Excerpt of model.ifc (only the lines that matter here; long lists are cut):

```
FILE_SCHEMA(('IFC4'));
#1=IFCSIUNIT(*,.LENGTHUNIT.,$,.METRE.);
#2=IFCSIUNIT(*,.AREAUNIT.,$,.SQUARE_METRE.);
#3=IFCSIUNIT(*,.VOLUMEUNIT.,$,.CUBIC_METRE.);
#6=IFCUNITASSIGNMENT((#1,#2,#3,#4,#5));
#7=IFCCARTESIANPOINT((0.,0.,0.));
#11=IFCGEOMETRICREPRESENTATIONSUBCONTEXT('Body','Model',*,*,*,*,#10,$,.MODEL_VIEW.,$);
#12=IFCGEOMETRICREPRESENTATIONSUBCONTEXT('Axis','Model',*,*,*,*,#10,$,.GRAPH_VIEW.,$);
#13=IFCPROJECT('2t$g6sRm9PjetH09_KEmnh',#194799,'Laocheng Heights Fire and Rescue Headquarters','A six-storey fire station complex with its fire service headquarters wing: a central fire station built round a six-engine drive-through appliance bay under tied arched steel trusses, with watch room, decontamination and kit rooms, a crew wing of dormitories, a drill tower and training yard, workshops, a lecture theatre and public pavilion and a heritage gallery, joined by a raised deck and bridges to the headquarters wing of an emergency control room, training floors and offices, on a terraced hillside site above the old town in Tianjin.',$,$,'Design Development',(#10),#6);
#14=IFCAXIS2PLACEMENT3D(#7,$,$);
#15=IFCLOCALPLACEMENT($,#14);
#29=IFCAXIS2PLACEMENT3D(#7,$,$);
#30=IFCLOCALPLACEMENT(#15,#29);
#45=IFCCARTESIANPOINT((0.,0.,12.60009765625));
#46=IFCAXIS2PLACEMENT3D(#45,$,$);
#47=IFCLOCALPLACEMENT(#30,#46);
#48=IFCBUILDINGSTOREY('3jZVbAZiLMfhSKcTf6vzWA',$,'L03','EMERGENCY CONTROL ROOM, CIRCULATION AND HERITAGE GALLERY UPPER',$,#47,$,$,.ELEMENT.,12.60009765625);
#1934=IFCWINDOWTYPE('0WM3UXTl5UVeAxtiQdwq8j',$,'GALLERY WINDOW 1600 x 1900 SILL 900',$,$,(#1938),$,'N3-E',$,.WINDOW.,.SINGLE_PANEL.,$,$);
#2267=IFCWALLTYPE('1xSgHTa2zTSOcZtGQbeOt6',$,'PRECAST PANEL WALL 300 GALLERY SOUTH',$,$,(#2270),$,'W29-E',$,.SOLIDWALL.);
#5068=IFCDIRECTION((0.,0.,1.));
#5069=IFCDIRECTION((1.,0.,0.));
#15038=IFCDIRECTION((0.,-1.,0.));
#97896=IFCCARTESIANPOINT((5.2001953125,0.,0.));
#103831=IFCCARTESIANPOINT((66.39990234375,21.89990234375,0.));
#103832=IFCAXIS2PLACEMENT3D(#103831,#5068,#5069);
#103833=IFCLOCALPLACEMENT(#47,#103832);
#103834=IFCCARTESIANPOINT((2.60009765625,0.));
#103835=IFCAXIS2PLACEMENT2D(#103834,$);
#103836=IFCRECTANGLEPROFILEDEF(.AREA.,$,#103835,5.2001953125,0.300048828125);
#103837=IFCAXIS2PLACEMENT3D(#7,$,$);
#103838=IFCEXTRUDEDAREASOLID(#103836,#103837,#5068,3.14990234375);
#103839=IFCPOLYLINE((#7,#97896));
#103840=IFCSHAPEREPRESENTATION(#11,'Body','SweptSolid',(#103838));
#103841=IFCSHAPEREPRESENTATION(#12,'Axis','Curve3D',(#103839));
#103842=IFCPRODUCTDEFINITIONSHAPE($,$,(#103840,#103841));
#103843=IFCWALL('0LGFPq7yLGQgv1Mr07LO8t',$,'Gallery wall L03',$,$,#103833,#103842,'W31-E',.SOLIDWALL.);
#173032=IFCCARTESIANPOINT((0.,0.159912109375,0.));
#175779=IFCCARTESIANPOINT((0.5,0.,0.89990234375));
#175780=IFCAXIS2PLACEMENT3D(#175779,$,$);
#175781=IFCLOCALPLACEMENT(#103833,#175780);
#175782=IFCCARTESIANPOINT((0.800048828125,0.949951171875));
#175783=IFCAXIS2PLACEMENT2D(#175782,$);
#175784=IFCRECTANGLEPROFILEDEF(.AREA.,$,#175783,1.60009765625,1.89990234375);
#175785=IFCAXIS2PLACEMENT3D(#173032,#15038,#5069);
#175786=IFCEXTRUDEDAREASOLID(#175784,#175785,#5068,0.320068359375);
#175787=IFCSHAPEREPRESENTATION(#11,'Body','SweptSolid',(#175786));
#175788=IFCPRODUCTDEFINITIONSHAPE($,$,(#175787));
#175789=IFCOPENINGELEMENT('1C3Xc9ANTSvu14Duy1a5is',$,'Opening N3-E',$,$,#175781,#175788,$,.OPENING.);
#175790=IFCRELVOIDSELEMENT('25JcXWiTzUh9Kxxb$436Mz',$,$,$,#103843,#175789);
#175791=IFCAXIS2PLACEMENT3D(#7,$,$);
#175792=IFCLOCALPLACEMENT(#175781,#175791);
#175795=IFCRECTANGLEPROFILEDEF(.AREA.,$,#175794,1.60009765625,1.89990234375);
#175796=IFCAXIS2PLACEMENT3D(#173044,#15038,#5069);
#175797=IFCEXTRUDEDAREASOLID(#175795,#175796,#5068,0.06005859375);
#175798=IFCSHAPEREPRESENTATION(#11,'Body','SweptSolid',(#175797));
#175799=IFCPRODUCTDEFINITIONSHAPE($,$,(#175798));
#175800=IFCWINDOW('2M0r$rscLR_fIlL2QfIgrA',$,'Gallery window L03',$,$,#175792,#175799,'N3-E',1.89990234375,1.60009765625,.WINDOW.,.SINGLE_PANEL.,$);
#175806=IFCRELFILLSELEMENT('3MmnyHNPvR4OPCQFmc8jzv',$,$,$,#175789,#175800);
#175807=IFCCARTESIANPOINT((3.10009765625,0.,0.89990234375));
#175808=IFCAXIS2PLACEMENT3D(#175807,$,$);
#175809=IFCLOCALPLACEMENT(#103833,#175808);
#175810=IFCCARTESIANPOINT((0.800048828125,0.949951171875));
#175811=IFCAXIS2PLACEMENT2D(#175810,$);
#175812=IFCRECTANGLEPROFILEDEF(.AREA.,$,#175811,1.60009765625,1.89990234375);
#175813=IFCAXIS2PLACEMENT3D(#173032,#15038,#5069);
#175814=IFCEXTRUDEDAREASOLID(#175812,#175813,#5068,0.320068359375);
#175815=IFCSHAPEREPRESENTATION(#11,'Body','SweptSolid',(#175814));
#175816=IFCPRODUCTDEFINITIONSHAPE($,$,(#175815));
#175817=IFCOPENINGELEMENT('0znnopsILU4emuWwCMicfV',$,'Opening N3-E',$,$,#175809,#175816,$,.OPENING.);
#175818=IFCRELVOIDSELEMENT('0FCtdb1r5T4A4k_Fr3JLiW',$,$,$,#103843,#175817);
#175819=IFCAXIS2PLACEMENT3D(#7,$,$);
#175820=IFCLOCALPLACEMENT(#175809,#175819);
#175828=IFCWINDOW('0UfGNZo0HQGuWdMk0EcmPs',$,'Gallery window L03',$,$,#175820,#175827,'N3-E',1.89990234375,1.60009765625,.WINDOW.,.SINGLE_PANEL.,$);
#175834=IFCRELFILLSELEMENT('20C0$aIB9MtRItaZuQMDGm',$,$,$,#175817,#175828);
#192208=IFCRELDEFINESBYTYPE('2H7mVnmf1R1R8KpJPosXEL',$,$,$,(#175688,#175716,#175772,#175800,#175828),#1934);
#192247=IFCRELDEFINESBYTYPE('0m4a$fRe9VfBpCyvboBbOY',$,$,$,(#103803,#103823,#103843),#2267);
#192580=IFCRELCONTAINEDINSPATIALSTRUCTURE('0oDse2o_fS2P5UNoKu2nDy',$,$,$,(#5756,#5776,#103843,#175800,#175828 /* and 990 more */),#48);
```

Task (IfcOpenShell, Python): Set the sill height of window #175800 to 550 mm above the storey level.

```python
import numpy as np
import ifcopenshell
import ifcopenshell.api.geometry
import ifcopenshell.geom
import ifcopenshell.util.element
import ifcopenshell.util.placement
import ifcopenshell.util.shape
import ifcopenshell.util.unit

model = ifcopenshell.open("model.ifc")
unit_scale = ifcopenshell.util.unit.calculate_unit_scale(model)

window = model.by_guid("2M0r$rscLR_fIlL2QfIgrA")
opening = window.FillsVoids[0].RelatingOpeningElement
storey = ifcopenshell.util.element.get_container(window, ifc_class="IfcBuildingStorey")
level = ifcopenshell.util.placement.get_local_placement(storey.ObjectPlacement)[2, 3]

# The opening's origin need not be at the sill, so measure its lowest point.
shape = ifcopenshell.geom.create_shape(ifcopenshell.geom.settings(), opening)
bottom = ifcopenshell.util.shape.get_shape_bottom_elevation(shape, shape.geometry) / unit_scale
dz = level + 0.55 - bottom

shift = np.array([0.0, 0.0, dz])
# The window is placed relative to its opening, so it follows when the opening moves.
matrix = ifcopenshell.util.placement.get_local_placement(opening.ObjectPlacement)
matrix[:3, 3] += shift
ifcopenshell.api.geometry.edit_object_placement(
    model, product=opening, matrix=matrix, is_si=False, should_transform_children=True
)

print(f"moved by {dz * unit_scale:+.3f} m")

model.write("model-out.ifc")
```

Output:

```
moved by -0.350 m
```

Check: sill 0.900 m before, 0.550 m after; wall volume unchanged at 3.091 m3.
